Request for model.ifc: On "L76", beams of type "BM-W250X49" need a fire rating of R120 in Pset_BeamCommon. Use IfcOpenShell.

First a look at what the model holds.

```python
import ifcopenshell
import ifcopenshell.util.element

model = ifcopenshell.open("model.ifc")
print(model.schema)
storey = next(s for s in model.by_type("IfcBuildingStorey") if s.Name == "L76")
beams = [e for e in ifcopenshell.util.element.get_decomposition(storey) if e.is_a("IfcBeam")]
seen = {}
for e in beams:
    element_type = ifcopenshell.util.element.get_type(e)
    key = (element_type.Name if element_type != e and element_type else None, ifcopenshell.util.element.get_pset(e, "Pset_BeamCommon", "FireRating"))
    seen[key] = seen.get(key, 0) + 1
for (name, value), count in sorted(seen.items(), key=str):
    print(count, "x", name, "|", value)
```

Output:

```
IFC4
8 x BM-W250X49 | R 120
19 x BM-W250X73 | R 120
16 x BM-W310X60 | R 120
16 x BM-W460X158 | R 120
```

```python
import ifcopenshell
import ifcopenshell.api.pset
import ifcopenshell.util.element

model = ifcopenshell.open("model.ifc")

storey = next(s for s in model.by_type("IfcBuildingStorey") if s.Name == "L76")
beams = [e for e in ifcopenshell.util.element.get_decomposition(storey) if e.is_a("IfcBeam")]

count = 0
for e in beams:
    element_type = ifcopenshell.util.element.get_type(e)
    if element_type in (None, e) or element_type.Name != "BM-W250X49":
        continue
    # add_pset returns the element's existing set when there is one.
    pset = ifcopenshell.api.pset.add_pset(model, product=e, name="Pset_BeamCommon")
    ifcopenshell.api.pset.edit_pset(model, pset=pset, properties={"FireRating": "R120"})
    count += 1

print(count, "beams updated")

model.write("model_rev.ifc")
```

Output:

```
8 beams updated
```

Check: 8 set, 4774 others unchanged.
